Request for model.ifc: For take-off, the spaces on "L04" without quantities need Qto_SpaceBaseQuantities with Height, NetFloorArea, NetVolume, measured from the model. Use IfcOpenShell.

First a look at what the model holds.

```python
import ifcopenshell
import ifcopenshell.util.element
import ifcopenshell.util.unit

model = ifcopenshell.open("model.ifc")
print(model.schema)
for unit_type in ("LENGTHUNIT", "AREAUNIT", "VOLUMEUNIT"):
    print(unit_type, ifcopenshell.util.unit.calculate_unit_scale(model, unit_type))
storey = next(s for s in model.by_type("IfcBuildingStorey") if s.Name == "L04")
spaces = [e for e in ifcopenshell.util.element.get_decomposition(storey) if e.is_a("IfcSpace")]
for e in sorted(spaces, key=lambda e: e.id()):
    print(e.id(), e.is_a(), e.Name, list(ifcopenshell.util.element.get_psets(e, qtos_only=True)), sep=" | ")
```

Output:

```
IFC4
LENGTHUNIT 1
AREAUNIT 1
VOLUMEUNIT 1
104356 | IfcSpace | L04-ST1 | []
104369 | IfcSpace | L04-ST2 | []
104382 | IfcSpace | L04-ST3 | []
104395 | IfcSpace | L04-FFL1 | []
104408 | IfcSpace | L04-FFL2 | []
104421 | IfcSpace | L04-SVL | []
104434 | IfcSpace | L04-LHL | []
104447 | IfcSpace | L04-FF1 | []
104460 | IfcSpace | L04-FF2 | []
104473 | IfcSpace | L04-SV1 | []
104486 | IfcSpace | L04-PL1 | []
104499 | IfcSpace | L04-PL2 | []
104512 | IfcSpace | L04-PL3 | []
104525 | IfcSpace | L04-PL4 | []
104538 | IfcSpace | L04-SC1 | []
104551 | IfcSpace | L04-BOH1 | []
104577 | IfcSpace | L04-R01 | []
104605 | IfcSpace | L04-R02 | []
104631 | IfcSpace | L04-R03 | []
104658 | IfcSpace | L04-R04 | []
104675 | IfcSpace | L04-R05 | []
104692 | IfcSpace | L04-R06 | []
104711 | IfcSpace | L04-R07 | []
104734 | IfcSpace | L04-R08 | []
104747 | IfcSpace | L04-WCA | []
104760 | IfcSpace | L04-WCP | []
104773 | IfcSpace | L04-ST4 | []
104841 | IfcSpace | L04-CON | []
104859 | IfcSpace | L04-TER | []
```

```python
import ifcopenshell
import ifcopenshell.api.pset
import ifcopenshell.geom
import ifcopenshell.util.element
import ifcopenshell.util.shape
import ifcopenshell.util.unit

model = ifcopenshell.open("model.ifc")
unit_scale = ifcopenshell.util.unit.calculate_unit_scale(model)
area_scale = ifcopenshell.util.unit.calculate_unit_scale(model, "AREAUNIT")
volume_scale = ifcopenshell.util.unit.calculate_unit_scale(model, "VOLUMEUNIT")
settings = ifcopenshell.geom.settings()

storey = next(s for s in model.by_type("IfcBuildingStorey") if s.Name == "L04")
spaces = [e for e in ifcopenshell.util.element.get_decomposition(storey) if e.is_a("IfcSpace")]

for e in sorted(spaces, key=lambda e: e.id()):
    if ifcopenshell.util.element.get_psets(e, qtos_only=True, should_inherit=False):
        continue
    # Geometry comes back in metres, in the element's own axes.
    shape = ifcopenshell.geom.create_shape(settings, e)
    values = {
        "Height": ifcopenshell.util.shape.get_z(shape.geometry) / unit_scale,
        "NetFloorArea": ifcopenshell.util.shape.get_footprint_area(shape.geometry) / area_scale,
        "NetVolume": ifcopenshell.util.shape.get_volume(shape.geometry) / volume_scale,
    }
    qto = ifcopenshell.api.pset.add_qto(model, product=e, name="Qto_SpaceBaseQuantities")
    ifcopenshell.api.pset.edit_qto(model, qto=qto, properties=values)
    print(e.id(), {k: round(v, 3) for k, v in values.items()})

model.write("model_updated.ifc")
```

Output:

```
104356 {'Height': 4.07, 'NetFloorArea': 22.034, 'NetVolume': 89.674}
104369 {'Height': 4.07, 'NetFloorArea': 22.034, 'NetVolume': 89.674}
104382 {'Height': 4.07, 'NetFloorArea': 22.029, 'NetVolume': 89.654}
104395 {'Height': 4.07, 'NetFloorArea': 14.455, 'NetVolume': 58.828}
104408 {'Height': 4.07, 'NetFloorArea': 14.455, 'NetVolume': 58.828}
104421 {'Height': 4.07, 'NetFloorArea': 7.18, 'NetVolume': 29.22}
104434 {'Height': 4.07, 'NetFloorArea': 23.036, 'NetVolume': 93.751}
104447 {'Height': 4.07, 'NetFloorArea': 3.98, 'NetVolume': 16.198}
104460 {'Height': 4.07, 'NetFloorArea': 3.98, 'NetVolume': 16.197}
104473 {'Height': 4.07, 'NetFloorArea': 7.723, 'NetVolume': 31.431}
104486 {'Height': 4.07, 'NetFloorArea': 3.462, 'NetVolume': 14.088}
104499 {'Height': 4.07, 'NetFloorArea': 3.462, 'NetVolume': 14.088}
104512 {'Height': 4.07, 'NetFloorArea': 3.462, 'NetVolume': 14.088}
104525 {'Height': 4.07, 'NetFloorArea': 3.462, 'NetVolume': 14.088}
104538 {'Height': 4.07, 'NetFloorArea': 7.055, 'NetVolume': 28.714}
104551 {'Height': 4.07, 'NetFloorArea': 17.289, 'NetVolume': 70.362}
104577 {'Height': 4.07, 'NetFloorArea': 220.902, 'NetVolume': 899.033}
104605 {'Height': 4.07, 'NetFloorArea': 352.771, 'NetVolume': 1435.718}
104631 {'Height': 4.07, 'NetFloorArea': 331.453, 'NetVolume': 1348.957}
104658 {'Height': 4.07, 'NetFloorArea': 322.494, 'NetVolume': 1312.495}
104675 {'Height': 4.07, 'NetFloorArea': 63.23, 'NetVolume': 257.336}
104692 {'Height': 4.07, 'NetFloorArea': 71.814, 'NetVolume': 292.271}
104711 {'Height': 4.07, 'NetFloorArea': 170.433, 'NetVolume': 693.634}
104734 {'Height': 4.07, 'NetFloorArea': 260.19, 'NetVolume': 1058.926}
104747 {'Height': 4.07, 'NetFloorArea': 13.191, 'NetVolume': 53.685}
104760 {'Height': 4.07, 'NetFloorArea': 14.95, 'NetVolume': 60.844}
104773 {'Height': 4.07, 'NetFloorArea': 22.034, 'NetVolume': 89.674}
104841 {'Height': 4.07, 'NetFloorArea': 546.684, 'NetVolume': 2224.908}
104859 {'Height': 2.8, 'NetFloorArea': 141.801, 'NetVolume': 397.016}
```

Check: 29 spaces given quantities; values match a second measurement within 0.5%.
